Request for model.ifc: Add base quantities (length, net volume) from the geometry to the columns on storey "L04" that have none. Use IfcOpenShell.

First a look at what the model holds.

```python
import ifcopenshell
import ifcopenshell.util.element
import ifcopenshell.util.unit

model = ifcopenshell.open("model.ifc")
print(model.schema)
for unit_type in ("LENGTHUNIT", "AREAUNIT", "VOLUMEUNIT"):
    print(unit_type, ifcopenshell.util.unit.calculate_unit_scale(model, unit_type))
storey = next(s for s in model.by_type("IfcBuildingStorey") if s.Name == "L04")
columns = [e for e in ifcopenshell.util.element.get_decomposition(storey) if e.is_a("IfcColumn")]
for e in sorted(columns, key=lambda e: e.id()):
    print(e.id(), e.is_a(), e.Name, list(ifcopenshell.util.element.get_psets(e, qtos_only=True)), sep=" | ")
```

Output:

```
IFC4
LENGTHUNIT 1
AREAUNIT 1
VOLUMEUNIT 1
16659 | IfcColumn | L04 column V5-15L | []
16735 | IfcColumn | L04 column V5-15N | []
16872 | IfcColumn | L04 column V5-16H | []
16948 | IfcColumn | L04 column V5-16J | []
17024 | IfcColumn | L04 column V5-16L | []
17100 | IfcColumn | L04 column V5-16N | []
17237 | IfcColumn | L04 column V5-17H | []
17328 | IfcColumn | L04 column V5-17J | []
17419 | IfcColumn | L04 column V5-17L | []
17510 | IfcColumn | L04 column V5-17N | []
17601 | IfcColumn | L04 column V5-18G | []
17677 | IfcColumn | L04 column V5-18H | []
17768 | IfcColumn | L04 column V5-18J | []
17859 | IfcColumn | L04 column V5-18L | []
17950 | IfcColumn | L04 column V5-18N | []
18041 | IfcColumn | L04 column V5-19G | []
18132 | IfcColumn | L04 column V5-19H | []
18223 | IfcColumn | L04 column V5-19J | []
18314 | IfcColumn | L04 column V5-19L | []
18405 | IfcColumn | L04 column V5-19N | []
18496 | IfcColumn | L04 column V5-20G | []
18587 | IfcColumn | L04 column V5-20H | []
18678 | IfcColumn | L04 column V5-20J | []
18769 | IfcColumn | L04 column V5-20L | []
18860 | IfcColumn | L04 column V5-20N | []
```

```python
import ifcopenshell
import ifcopenshell.api.pset
import ifcopenshell.geom
import ifcopenshell.util.element
import ifcopenshell.util.shape
import ifcopenshell.util.unit

model = ifcopenshell.open("model.ifc")
unit_scale = ifcopenshell.util.unit.calculate_unit_scale(model)
volume_scale = ifcopenshell.util.unit.calculate_unit_scale(model, "VOLUMEUNIT")
settings = ifcopenshell.geom.settings()

storey = next(s for s in model.by_type("IfcBuildingStorey") if s.Name == "L04")
columns = [e for e in ifcopenshell.util.element.get_decomposition(storey) if e.is_a("IfcColumn")]

for e in sorted(columns, key=lambda e: e.id()):
    if ifcopenshell.util.element.get_psets(e, qtos_only=True, should_inherit=False):
        continue
    # Geometry comes back in metres, in the element's own axes.
    shape = ifcopenshell.geom.create_shape(settings, e)
    values = {
        "Length": ifcopenshell.util.shape.get_z(shape.geometry) / unit_scale,
        "NetVolume": ifcopenshell.util.shape.get_volume(shape.geometry) / volume_scale,
    }
    qto = ifcopenshell.api.pset.add_qto(model, product=e, name="Qto_ColumnBaseQuantities")
    ifcopenshell.api.pset.edit_qto(model, qto=qto, properties=values)
    print(e.id(), {k: round(v, 3) for k, v in values.items()})

model.write("model_updated.ifc")
```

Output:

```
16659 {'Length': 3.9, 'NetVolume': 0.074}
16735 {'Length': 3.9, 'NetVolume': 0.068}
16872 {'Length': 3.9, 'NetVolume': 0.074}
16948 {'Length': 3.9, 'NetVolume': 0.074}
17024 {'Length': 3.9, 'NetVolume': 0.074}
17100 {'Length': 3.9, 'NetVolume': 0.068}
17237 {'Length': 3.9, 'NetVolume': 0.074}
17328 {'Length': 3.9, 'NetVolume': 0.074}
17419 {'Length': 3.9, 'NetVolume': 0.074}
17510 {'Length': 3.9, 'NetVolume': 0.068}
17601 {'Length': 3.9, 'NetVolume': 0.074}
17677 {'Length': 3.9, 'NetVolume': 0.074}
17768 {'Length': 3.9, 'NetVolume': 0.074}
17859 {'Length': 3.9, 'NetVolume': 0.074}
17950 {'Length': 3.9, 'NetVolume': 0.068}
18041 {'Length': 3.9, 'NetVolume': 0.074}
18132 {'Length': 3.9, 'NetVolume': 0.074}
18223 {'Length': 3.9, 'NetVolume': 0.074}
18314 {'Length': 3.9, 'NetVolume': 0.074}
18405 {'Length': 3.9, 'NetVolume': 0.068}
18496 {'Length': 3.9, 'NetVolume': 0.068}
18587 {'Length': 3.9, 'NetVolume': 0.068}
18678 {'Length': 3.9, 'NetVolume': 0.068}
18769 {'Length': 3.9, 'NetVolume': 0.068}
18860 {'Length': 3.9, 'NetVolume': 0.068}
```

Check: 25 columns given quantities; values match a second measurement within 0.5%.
